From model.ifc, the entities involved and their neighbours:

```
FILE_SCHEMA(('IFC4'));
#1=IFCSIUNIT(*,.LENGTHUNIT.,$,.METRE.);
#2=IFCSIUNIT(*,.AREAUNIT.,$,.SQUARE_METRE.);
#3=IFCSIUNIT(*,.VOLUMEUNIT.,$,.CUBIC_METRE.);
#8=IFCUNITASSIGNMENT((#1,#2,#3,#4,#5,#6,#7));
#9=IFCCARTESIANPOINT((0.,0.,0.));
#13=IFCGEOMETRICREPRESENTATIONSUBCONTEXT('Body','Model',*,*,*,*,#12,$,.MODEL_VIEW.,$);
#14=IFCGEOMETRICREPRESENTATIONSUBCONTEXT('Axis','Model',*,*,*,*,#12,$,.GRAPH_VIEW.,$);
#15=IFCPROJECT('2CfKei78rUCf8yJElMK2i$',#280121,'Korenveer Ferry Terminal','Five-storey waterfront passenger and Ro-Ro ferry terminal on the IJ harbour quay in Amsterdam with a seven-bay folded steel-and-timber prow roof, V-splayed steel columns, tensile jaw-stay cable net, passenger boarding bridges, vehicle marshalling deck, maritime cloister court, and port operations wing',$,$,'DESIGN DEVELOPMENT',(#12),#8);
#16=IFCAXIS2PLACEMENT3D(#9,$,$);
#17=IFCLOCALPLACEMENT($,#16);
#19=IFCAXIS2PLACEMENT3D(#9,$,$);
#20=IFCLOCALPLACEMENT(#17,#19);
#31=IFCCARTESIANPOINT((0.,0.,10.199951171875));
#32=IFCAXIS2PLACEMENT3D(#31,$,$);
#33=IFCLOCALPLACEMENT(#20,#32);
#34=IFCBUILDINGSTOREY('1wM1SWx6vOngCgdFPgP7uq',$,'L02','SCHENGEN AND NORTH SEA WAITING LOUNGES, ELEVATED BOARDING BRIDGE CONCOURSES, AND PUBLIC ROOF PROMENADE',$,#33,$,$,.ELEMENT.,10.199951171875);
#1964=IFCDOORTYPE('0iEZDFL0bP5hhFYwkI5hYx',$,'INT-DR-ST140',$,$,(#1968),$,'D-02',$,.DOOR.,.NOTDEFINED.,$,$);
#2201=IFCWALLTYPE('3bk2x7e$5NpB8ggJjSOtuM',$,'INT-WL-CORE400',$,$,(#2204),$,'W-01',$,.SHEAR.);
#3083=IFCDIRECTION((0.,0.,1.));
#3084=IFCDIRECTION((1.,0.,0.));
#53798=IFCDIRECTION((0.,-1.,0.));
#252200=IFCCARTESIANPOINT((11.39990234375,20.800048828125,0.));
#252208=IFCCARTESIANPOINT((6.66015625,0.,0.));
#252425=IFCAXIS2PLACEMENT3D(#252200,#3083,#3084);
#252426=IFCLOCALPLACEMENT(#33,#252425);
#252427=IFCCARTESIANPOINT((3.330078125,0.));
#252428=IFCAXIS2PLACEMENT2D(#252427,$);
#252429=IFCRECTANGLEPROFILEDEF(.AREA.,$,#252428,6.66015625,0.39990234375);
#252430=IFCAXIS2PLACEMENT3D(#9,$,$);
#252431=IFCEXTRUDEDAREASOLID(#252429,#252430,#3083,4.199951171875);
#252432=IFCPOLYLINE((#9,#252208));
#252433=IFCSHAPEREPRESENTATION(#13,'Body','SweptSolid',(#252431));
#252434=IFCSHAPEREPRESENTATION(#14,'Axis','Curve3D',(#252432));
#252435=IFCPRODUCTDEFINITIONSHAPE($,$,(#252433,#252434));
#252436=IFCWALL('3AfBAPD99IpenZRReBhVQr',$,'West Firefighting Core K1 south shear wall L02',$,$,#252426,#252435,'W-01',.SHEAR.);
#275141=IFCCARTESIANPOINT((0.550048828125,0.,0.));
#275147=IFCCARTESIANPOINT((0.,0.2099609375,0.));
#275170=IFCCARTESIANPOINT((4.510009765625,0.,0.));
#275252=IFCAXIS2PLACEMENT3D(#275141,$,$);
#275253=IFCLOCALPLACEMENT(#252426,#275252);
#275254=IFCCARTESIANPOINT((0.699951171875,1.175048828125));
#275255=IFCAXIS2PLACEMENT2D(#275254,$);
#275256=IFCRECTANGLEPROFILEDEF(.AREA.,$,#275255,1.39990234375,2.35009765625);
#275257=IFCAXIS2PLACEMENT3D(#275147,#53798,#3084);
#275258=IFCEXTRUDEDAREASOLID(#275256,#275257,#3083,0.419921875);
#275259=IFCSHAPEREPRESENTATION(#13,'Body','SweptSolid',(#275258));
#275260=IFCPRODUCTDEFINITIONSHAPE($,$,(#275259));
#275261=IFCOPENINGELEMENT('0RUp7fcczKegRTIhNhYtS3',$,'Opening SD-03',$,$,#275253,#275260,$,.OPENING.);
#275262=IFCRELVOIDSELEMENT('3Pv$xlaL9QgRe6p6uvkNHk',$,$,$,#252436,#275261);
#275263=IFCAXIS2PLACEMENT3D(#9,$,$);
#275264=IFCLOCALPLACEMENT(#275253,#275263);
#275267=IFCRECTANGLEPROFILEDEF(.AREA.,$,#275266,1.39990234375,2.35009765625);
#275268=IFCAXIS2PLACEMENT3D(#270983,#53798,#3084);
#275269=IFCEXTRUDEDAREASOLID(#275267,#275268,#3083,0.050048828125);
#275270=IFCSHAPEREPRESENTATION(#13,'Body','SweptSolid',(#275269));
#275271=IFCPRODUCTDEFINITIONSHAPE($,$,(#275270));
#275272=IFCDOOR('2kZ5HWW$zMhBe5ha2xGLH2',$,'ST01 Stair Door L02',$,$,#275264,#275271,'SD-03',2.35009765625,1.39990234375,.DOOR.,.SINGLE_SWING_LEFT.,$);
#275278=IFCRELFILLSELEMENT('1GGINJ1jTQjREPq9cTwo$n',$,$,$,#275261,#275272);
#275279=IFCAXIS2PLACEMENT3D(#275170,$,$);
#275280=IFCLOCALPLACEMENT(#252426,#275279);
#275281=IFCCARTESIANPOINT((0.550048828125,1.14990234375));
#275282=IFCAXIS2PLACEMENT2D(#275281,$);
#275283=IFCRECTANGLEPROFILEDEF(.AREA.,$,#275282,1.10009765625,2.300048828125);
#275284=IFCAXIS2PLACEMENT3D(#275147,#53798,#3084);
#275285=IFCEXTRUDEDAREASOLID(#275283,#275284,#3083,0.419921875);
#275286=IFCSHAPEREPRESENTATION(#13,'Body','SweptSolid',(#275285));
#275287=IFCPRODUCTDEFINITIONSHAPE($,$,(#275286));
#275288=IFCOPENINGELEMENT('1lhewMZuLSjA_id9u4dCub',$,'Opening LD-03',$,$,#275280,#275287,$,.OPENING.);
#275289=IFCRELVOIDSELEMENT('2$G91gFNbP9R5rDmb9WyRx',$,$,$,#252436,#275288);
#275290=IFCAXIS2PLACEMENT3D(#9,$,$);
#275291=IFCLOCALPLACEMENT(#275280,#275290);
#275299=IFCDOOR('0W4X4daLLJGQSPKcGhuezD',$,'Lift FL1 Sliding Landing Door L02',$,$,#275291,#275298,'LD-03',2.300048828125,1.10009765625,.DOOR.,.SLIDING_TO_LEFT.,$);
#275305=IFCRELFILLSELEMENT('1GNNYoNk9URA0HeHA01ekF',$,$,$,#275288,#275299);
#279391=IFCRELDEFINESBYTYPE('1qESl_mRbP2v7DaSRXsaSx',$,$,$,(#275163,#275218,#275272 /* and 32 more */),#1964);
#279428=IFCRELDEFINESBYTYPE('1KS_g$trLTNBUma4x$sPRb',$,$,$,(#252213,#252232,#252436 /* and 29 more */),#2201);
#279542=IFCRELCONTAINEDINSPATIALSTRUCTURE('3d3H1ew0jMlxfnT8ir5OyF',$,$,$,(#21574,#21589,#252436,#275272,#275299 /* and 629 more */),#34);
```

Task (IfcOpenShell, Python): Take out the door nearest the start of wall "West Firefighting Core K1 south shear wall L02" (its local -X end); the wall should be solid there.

```python
import ifcopenshell
import ifcopenshell.api.feature
import ifcopenshell.api.root
import ifcopenshell.geom
import ifcopenshell.util.shape

model = ifcopenshell.open("model.ifc")
settings = ifcopenshell.geom.settings()


def volume(element):
    """Net volume in cubic metres, openings subtracted."""
    shape = ifcopenshell.geom.create_shape(settings, element)
    return ifcopenshell.util.shape.get_volume(shape.geometry)


door = model.by_guid("2kZ5HWW$zMhBe5ha2xGLH2")
opening = door.FillsVoids[0].RelatingOpeningElement
wall = opening.VoidsElements[0].RelatingBuildingElement
before = volume(wall)

ifcopenshell.api.root.remove_product(model, product=door)
ifcopenshell.api.feature.remove_feature(model, feature=opening)

after = volume(wall)

print(f"wall volume {before:.3f} -> {after:.3f} m3")

model.write("model_v2.ifc")
```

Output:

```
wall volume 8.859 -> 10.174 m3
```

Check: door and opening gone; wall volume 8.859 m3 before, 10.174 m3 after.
